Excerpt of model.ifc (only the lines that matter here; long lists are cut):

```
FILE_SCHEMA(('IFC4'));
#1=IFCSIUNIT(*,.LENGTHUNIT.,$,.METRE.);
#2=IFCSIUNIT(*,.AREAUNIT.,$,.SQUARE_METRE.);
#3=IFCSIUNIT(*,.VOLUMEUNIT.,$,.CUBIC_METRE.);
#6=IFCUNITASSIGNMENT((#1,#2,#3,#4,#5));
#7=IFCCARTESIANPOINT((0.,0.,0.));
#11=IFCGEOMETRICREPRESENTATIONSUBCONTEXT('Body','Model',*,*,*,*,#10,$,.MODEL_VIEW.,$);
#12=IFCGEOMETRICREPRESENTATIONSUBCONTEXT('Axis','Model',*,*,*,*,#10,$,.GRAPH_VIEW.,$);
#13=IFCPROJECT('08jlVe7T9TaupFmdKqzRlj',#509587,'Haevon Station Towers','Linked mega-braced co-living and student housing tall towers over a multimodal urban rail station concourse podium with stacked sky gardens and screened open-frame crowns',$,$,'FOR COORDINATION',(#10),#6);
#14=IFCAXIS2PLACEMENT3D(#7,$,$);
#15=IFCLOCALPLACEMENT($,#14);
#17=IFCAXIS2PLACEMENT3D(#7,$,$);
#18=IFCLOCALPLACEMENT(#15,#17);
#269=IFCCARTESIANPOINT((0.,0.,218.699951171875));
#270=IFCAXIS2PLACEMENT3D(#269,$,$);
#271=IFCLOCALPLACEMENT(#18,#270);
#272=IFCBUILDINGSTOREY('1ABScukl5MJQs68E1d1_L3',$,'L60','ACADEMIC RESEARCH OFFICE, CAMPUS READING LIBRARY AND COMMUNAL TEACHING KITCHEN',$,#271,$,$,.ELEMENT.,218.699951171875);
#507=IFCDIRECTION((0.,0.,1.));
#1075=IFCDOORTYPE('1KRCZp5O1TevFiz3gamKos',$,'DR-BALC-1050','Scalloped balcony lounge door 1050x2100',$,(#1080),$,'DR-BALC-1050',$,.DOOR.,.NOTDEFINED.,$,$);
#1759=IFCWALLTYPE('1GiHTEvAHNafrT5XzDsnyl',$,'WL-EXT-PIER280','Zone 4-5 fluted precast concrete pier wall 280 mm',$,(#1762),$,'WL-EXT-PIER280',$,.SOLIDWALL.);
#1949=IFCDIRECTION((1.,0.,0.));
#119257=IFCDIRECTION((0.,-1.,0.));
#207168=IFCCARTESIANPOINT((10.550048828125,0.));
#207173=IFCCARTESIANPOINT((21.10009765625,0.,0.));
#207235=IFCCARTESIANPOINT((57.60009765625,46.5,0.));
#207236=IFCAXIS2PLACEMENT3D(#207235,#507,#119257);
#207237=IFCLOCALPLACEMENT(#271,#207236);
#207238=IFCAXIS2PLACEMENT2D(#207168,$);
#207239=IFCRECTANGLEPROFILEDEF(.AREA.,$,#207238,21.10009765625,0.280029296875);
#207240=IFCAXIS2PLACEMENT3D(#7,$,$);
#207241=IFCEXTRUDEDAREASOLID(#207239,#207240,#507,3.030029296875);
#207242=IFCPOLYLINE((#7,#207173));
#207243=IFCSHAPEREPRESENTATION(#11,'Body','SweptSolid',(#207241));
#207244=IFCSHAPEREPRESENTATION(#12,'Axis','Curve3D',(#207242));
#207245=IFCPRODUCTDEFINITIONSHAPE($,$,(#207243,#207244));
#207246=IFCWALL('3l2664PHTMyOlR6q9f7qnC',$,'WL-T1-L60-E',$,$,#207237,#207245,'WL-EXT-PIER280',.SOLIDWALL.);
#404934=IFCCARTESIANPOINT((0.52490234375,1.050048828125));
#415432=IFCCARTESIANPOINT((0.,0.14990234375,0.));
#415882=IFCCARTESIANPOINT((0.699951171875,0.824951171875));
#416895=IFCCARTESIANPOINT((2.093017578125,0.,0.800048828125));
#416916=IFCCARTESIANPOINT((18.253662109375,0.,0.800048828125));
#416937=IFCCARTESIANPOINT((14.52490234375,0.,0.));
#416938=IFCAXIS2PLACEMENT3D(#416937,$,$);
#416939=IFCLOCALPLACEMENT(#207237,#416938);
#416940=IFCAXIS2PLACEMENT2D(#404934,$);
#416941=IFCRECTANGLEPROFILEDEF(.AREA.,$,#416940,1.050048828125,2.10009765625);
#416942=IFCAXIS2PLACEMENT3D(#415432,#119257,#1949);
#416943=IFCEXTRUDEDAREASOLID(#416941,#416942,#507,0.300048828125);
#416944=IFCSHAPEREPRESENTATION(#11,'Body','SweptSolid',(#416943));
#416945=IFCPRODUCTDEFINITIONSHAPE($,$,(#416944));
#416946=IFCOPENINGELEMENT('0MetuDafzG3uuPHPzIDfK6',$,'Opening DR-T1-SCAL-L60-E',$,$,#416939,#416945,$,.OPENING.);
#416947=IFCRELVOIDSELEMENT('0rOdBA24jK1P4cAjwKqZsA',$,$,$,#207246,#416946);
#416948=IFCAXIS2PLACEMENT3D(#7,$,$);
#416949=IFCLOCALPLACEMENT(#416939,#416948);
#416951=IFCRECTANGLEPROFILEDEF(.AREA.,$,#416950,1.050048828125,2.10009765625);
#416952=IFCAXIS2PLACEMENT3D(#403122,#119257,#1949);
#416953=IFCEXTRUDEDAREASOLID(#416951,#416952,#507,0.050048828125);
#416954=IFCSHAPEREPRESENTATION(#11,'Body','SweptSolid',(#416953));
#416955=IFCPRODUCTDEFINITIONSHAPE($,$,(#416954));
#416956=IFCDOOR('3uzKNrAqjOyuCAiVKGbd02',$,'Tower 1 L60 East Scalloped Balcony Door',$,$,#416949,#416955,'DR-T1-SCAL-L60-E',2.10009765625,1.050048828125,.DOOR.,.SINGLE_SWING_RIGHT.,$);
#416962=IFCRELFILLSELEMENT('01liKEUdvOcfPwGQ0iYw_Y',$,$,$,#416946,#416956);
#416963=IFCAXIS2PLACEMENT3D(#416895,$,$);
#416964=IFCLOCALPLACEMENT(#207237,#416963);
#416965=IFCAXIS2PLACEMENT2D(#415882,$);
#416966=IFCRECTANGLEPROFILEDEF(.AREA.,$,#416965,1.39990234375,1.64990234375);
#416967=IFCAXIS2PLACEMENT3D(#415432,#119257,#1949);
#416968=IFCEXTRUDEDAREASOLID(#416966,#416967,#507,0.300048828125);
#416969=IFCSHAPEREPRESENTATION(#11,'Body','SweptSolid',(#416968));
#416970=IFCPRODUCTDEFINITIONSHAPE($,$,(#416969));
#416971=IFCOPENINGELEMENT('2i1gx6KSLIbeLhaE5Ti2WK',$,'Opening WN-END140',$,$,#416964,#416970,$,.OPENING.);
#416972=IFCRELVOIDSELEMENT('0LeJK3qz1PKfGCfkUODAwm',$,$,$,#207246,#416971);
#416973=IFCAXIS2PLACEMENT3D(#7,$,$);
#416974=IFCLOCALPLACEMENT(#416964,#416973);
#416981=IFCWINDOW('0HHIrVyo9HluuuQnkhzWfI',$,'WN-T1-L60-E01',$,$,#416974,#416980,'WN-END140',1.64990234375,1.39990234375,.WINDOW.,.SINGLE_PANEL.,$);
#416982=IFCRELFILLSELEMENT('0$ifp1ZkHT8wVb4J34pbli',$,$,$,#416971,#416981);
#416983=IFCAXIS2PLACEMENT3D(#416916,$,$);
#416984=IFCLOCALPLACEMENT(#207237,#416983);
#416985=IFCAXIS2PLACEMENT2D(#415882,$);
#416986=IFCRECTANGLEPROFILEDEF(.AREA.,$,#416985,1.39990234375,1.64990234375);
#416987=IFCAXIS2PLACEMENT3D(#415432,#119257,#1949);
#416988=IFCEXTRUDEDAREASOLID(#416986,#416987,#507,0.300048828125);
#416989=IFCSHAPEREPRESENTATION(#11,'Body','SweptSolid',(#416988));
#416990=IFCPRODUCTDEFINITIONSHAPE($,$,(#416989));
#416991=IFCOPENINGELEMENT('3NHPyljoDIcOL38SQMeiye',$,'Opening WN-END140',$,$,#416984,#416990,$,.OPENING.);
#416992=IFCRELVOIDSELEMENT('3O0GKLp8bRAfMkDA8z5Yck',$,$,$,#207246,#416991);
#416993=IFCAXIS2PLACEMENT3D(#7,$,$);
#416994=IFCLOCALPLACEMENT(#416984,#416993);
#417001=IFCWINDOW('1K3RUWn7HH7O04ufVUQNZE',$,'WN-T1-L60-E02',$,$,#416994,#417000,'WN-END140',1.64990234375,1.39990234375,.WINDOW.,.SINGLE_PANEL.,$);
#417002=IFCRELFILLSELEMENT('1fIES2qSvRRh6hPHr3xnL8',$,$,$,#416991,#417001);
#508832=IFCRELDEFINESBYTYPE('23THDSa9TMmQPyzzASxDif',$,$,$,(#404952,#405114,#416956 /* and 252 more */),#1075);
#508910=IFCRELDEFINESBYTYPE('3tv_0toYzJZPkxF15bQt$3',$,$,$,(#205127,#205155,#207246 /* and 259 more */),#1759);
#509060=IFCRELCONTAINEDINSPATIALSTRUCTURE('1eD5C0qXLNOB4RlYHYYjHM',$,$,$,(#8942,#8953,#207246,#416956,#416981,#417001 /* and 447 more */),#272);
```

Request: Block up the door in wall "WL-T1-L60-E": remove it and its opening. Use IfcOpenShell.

```python
import ifcopenshell
import ifcopenshell.api.feature
import ifcopenshell.api.root
import ifcopenshell.geom
import ifcopenshell.util.shape

model = ifcopenshell.open("model.ifc")
settings = ifcopenshell.geom.settings()


def volume(element):
    """Net volume in cubic metres, openings subtracted."""
    shape = ifcopenshell.geom.create_shape(settings, element)
    return ifcopenshell.util.shape.get_volume(shape.geometry)


door = model.by_id(416956)
opening = door.FillsVoids[0].RelatingOpeningElement
wall = opening.VoidsElements[0].RelatingBuildingElement
before = volume(wall)

ifcopenshell.api.root.remove_product(model, product=door)
ifcopenshell.api.feature.remove_feature(model, feature=opening)

after = volume(wall)

print(f"wall volume {before:.3f} -> {after:.3f} m3")

model.write("model-out.ifc")
```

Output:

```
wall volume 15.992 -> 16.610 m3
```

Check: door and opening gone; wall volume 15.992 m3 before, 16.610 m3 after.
